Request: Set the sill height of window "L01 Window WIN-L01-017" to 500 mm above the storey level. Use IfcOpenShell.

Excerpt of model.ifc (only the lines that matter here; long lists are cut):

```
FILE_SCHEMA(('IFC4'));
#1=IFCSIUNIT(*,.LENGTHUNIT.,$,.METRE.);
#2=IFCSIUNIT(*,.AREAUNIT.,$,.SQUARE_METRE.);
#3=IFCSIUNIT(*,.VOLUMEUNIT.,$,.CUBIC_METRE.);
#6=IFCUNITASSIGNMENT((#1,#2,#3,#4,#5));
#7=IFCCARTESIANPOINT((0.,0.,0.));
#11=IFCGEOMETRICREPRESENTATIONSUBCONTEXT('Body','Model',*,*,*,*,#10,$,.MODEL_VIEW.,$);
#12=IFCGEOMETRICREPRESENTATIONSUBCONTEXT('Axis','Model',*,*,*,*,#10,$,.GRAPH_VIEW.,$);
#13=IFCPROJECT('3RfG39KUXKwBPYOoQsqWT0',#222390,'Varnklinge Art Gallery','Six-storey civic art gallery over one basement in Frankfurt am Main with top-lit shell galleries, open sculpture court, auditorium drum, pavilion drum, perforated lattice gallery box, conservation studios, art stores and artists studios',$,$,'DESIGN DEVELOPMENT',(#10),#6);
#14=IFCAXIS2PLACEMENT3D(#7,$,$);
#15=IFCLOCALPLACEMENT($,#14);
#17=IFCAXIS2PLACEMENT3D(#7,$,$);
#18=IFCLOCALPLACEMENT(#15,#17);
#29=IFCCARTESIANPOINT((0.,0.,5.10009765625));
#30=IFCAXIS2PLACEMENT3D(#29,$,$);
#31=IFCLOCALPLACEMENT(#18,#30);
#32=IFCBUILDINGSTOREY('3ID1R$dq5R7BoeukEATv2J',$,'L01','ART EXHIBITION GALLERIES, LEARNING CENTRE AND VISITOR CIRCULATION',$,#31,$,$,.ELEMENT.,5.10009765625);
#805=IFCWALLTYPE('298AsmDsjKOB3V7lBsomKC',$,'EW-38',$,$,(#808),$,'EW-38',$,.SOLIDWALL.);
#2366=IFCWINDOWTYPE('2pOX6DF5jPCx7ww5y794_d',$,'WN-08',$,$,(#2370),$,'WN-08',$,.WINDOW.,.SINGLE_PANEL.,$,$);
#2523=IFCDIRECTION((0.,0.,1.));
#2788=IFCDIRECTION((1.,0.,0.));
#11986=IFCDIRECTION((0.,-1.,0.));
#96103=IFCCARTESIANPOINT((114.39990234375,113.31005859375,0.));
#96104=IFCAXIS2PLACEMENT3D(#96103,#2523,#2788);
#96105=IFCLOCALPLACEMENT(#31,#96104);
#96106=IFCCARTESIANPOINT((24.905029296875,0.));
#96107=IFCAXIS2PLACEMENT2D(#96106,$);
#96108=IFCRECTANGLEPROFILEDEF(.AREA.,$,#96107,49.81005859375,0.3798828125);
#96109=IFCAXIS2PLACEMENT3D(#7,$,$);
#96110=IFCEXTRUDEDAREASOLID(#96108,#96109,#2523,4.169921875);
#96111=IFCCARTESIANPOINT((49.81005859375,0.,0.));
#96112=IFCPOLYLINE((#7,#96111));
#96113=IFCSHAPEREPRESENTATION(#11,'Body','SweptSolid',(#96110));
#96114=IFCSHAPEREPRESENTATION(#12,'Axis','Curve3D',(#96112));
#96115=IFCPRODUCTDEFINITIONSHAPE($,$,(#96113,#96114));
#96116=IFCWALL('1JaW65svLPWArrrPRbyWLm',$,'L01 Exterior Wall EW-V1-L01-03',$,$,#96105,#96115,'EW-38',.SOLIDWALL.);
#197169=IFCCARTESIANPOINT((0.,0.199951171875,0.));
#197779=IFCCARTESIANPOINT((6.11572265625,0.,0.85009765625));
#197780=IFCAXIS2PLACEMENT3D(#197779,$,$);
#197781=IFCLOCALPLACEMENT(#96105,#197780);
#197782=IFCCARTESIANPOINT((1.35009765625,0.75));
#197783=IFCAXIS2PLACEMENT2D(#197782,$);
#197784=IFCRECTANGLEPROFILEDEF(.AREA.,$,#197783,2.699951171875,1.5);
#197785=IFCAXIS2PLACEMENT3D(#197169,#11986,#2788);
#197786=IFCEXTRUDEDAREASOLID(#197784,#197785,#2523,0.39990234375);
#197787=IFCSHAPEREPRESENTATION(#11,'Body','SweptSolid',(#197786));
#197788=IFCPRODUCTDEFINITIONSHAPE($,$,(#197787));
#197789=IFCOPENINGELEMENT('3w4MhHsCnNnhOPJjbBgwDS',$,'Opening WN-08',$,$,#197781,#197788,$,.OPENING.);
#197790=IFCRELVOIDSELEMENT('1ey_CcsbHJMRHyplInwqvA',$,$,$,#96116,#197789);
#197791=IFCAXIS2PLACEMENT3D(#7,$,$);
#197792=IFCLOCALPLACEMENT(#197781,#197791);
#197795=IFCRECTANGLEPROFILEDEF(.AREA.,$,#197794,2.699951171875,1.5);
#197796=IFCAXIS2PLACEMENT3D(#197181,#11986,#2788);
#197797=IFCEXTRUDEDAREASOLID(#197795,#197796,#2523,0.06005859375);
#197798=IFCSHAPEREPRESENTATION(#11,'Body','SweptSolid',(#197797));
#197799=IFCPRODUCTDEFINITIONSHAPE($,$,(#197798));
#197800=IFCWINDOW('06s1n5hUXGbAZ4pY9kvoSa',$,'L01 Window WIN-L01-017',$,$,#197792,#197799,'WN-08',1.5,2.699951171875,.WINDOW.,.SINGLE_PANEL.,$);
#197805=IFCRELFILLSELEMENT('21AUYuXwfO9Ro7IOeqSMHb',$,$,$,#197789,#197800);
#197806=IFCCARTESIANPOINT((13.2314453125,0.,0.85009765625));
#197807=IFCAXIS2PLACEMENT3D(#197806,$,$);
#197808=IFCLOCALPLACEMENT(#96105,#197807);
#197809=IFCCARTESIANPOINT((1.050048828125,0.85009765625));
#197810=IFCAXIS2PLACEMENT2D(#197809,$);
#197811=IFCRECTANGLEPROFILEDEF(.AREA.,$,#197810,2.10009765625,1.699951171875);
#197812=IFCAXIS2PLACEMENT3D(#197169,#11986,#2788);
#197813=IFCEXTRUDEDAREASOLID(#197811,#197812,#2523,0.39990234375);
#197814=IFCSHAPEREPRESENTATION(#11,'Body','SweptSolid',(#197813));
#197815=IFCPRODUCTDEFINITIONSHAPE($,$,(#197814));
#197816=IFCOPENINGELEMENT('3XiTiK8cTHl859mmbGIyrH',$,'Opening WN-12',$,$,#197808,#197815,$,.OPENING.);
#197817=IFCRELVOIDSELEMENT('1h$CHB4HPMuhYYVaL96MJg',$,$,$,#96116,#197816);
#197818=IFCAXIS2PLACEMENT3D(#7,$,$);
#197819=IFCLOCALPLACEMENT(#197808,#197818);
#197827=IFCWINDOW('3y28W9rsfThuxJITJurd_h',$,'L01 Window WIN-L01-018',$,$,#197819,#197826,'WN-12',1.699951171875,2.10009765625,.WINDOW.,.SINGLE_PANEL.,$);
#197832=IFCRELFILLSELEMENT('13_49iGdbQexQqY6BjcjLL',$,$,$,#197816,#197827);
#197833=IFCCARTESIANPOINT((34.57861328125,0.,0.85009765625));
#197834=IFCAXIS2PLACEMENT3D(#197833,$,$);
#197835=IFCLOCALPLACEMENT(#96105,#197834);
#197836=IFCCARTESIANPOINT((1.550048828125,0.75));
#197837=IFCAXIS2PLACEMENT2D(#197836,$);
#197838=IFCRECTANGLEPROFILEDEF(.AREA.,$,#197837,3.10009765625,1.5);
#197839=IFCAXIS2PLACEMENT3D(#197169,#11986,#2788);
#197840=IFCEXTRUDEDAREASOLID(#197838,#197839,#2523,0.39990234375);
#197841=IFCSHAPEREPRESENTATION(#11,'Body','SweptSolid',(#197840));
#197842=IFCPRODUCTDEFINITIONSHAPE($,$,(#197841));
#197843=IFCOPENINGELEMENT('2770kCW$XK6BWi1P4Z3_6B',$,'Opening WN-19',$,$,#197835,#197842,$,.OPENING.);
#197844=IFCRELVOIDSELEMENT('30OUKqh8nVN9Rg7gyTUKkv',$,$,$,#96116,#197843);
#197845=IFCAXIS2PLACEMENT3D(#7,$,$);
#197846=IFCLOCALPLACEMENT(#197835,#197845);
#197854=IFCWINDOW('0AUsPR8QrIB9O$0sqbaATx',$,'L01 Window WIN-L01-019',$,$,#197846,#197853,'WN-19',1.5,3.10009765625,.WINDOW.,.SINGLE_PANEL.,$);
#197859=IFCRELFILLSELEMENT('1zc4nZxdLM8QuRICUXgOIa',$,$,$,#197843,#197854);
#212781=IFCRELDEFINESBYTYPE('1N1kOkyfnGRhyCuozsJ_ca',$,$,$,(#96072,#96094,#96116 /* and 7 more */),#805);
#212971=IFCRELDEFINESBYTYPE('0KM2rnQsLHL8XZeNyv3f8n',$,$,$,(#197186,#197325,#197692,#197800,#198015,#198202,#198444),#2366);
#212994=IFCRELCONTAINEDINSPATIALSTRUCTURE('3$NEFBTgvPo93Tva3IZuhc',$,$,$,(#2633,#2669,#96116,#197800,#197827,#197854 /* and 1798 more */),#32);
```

```python
import numpy as np
import ifcopenshell
import ifcopenshell.api.geometry
import ifcopenshell.geom
import ifcopenshell.util.element
import ifcopenshell.util.placement
import ifcopenshell.util.shape
import ifcopenshell.util.unit

model = ifcopenshell.open("model.ifc")
unit_scale = ifcopenshell.util.unit.calculate_unit_scale(model)

window = model.by_guid("06s1n5hUXGbAZ4pY9kvoSa")
opening = window.FillsVoids[0].RelatingOpeningElement
storey = ifcopenshell.util.element.get_container(window, ifc_class="IfcBuildingStorey")
level = ifcopenshell.util.placement.get_local_placement(storey.ObjectPlacement)[2, 3]

# The opening's origin need not be at the sill, so measure its lowest point.
shape = ifcopenshell.geom.create_shape(ifcopenshell.geom.settings(), opening)
bottom = ifcopenshell.util.shape.get_shape_bottom_elevation(shape, shape.geometry) / unit_scale
dz = level + 0.5 / unit_scale - bottom

shift = np.array([0.0, 0.0, dz])
# The window is placed relative to its opening, so it follows when the opening moves.
matrix = ifcopenshell.util.placement.get_local_placement(opening.ObjectPlacement)
matrix[:3, 3] += shift
ifcopenshell.api.geometry.edit_object_placement(
    model, product=opening, matrix=matrix, is_si=False, should_transform_children=True
)

print(f"moved by {dz * unit_scale:+.3f} m")

model.write("model-out.ifc")
```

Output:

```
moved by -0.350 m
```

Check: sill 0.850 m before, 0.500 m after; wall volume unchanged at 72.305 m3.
